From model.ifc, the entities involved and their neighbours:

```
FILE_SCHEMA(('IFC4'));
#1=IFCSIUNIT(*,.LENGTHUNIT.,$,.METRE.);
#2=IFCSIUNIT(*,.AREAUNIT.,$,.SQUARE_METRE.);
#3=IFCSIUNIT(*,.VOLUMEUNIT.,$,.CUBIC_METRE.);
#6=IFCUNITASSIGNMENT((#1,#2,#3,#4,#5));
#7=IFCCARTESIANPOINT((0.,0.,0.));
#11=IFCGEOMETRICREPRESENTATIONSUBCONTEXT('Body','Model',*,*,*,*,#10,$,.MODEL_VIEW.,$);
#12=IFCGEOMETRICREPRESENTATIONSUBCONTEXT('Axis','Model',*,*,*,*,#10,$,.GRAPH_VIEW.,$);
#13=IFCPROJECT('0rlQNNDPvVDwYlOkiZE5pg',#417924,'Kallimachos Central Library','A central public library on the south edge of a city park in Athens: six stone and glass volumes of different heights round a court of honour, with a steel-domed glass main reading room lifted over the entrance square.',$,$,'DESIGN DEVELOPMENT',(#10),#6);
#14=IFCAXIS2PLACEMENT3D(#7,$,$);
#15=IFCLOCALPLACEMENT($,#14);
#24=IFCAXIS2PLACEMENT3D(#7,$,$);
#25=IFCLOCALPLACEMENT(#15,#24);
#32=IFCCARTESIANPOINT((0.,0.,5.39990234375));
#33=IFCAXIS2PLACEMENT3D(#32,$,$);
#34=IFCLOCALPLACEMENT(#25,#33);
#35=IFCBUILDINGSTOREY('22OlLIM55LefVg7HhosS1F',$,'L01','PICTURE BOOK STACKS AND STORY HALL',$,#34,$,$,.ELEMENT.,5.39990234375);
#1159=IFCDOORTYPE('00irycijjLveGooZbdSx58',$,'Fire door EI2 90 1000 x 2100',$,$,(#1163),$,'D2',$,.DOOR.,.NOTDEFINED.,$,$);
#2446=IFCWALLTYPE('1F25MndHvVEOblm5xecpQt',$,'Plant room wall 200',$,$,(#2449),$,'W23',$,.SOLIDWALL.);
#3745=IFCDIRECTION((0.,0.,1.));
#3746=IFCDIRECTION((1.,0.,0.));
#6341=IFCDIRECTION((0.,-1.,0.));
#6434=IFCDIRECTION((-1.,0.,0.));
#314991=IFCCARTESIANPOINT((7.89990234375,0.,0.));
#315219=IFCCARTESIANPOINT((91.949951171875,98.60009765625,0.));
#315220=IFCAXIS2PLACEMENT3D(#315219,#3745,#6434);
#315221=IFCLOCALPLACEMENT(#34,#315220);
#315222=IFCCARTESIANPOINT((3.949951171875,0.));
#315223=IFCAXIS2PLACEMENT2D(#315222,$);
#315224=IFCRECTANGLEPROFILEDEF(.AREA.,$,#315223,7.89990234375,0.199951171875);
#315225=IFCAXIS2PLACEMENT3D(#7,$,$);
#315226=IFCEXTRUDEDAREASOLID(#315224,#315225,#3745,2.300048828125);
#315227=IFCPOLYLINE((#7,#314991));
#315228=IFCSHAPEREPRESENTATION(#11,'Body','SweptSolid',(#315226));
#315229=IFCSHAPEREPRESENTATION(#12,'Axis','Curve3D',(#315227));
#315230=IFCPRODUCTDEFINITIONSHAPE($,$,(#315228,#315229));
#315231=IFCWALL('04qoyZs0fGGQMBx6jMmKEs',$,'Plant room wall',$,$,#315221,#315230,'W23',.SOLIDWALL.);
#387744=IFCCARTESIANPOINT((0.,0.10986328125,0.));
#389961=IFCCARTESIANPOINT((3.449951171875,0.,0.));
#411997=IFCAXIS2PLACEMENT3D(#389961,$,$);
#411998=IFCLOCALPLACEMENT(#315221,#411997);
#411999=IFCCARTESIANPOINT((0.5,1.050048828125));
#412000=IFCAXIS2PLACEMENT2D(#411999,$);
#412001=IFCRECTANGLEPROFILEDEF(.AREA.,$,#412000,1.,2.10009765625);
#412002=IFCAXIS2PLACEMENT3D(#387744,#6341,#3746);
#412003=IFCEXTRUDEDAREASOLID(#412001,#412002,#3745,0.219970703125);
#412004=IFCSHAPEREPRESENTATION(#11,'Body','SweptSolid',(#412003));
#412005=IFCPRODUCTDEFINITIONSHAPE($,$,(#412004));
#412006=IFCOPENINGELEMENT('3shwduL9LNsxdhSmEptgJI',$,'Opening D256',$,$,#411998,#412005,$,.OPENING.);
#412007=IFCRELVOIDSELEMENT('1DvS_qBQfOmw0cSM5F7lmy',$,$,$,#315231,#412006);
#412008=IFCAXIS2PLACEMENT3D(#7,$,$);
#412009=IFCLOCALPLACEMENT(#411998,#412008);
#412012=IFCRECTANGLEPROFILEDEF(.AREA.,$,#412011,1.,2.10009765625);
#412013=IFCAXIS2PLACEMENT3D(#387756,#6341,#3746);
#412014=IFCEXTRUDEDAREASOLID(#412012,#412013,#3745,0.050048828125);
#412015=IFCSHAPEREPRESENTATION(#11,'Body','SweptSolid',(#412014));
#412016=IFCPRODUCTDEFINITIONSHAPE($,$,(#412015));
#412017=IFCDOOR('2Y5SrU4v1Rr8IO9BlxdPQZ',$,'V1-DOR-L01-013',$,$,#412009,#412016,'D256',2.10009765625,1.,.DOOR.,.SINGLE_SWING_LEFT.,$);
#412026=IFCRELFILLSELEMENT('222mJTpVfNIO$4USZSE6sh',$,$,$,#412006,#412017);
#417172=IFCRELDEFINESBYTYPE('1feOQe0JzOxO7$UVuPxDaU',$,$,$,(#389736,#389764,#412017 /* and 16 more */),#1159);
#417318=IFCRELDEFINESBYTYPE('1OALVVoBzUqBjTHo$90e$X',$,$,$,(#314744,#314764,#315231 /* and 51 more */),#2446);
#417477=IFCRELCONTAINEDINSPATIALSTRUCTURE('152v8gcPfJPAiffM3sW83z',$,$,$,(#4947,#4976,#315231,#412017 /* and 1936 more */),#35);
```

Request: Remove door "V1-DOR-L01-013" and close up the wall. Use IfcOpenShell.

```python
import ifcopenshell
import ifcopenshell.api.feature
import ifcopenshell.api.root
import ifcopenshell.geom
import ifcopenshell.util.shape

model = ifcopenshell.open("model.ifc")
settings = ifcopenshell.geom.settings()


def volume(element):
    """Net volume in cubic metres, openings subtracted."""
    shape = ifcopenshell.geom.create_shape(settings, element)
    return ifcopenshell.util.shape.get_volume(shape.geometry)


door = model.by_id(412017)
opening = door.FillsVoids[0].RelatingOpeningElement
wall = opening.VoidsElements[0].RelatingBuildingElement
before = volume(wall)

ifcopenshell.api.root.remove_product(model, product=door)
ifcopenshell.api.feature.remove_feature(model, feature=opening)

after = volume(wall)

print(f"wall volume {before:.3f} -> {after:.3f} m3")

model.write("model_updated.ifc")
```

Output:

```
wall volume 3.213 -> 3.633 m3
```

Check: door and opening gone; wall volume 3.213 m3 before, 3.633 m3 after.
